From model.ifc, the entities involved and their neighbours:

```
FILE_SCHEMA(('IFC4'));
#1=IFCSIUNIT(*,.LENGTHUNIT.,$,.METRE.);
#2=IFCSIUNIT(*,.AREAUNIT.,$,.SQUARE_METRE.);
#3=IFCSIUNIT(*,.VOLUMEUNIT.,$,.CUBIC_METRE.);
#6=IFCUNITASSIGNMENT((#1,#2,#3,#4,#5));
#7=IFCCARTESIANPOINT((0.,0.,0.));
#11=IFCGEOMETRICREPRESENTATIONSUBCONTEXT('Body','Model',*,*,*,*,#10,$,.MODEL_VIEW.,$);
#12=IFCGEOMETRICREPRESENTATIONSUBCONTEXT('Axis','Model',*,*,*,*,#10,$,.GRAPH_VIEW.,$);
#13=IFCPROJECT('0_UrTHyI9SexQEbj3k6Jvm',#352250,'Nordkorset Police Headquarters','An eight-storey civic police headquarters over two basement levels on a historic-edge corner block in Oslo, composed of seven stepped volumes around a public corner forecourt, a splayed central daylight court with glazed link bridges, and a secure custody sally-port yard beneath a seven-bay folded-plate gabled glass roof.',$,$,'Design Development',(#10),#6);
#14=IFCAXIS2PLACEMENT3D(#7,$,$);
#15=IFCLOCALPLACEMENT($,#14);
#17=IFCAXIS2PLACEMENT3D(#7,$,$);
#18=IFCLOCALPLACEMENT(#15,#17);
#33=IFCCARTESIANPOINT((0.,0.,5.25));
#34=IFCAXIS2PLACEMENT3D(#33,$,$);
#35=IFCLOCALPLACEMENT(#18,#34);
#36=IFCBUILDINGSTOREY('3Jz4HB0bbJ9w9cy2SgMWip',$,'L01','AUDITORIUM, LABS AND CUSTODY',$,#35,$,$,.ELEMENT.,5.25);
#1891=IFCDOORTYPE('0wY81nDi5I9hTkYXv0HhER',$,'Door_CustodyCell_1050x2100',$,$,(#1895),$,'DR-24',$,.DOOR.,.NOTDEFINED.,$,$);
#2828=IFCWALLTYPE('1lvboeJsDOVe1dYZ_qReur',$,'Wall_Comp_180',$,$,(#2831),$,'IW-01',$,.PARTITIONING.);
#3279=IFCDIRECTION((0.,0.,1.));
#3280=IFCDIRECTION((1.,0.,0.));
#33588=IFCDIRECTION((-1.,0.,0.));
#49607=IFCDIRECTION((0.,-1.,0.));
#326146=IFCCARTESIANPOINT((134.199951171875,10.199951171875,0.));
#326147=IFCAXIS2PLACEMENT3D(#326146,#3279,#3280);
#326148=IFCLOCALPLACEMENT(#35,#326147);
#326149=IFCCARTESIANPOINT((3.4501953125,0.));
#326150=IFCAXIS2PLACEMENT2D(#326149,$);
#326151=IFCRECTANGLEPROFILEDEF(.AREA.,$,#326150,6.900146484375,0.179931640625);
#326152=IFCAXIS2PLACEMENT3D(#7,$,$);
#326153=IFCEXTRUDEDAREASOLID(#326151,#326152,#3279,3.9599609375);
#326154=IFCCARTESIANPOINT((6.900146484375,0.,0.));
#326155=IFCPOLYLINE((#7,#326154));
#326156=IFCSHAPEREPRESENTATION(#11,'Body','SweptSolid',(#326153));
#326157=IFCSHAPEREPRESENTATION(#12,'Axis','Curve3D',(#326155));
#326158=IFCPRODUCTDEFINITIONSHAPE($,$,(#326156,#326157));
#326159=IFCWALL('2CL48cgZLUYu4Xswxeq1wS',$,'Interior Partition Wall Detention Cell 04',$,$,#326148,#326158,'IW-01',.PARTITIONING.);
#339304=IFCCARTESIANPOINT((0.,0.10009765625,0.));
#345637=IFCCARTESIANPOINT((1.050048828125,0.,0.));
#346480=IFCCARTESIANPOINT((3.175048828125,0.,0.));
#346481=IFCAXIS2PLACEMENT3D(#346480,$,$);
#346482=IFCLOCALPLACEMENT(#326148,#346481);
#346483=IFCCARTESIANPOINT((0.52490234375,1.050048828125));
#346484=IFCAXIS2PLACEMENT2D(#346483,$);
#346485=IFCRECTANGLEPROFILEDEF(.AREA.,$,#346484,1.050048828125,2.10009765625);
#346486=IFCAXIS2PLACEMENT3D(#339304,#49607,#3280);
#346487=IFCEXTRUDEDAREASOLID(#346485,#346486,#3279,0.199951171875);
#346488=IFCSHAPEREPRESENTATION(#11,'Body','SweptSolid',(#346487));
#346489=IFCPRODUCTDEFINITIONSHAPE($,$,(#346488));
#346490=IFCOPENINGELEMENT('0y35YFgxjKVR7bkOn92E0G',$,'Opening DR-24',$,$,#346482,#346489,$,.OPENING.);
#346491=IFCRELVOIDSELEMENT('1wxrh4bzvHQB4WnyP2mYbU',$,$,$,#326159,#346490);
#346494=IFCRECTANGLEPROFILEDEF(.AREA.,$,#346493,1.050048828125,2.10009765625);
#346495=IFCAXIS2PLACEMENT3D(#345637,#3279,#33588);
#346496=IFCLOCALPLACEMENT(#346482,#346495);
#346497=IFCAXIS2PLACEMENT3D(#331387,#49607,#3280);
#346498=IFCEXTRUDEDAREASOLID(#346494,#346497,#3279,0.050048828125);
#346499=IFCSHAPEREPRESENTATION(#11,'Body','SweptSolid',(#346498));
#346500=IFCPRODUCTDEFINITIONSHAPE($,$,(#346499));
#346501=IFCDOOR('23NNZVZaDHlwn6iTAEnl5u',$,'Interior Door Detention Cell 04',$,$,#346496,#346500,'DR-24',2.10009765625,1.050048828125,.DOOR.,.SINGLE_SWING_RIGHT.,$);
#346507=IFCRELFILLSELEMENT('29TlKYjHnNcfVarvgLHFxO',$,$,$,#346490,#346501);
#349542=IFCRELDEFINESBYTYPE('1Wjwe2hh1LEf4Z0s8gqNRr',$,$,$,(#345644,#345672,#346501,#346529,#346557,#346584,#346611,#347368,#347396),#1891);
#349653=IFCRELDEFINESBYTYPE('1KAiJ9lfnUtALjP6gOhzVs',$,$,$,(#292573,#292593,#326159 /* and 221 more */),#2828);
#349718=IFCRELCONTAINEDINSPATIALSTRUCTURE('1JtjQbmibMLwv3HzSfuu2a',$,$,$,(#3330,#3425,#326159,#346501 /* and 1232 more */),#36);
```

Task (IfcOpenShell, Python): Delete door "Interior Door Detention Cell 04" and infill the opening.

```python
import ifcopenshell
import ifcopenshell.api.feature
import ifcopenshell.api.root
import ifcopenshell.geom
import ifcopenshell.util.shape

model = ifcopenshell.open("model.ifc")
settings = ifcopenshell.geom.settings()


def volume(element):
    """Net volume in cubic metres, openings subtracted."""
    shape = ifcopenshell.geom.create_shape(settings, element)
    return ifcopenshell.util.shape.get_volume(shape.geometry)


door = model.by_id(346501)
opening = door.FillsVoids[0].RelatingOpeningElement
wall = opening.VoidsElements[0].RelatingBuildingElement
before = volume(wall)

ifcopenshell.api.root.remove_product(model, product=door)
ifcopenshell.api.feature.remove_feature(model, feature=opening)

after = volume(wall)

print(f"wall volume {before:.3f} -> {after:.3f} m3")

model.write("model_rev.ifc")
```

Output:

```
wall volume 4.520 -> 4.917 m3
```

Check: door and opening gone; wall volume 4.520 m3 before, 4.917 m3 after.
